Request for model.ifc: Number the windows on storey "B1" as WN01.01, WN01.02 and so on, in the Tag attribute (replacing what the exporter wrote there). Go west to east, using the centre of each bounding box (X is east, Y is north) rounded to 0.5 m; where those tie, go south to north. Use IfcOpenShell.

First a look at what the model holds.

```python
import ifcopenshell
import ifcopenshell.util.element
import ifcopenshell.util.placement

model = ifcopenshell.open("model.ifc")
print(model.schema)
storey = next(s for s in model.by_type("IfcBuildingStorey") if s.Name == "B1")
windows = [e for e in ifcopenshell.util.element.get_decomposition(storey) if e.is_a("IfcWindow")]
for e in sorted(windows, key=lambda e: e.id()):
    origin = ifcopenshell.util.placement.get_local_placement(e.ObjectPlacement)[:3, 3]
    print(e.id(), e.Tag, e.Name, origin.round(2) + 0.0, sep=" | ")
```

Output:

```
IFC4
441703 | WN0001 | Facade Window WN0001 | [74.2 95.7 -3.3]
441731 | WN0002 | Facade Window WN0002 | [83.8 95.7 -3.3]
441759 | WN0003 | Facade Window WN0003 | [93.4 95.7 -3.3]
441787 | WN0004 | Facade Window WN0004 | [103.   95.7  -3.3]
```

```python
import ifcopenshell
import ifcopenshell.geom
import ifcopenshell.util.element
import ifcopenshell.util.shape

model = ifcopenshell.open("model.ifc")
settings = ifcopenshell.geom.settings()
settings.set("use-world-coords", True)


def centre(element):
    shape = ifcopenshell.geom.create_shape(settings, element)
    return ifcopenshell.util.shape.get_bbox_centroid(shape.geometry)


storey = next(s for s in model.by_type("IfcBuildingStorey") if s.Name == "B1")
windows = [e for e in ifcopenshell.util.element.get_decomposition(storey) if e.is_a("IfcWindow")]

# Insertion points can sit at a corner or the storey origin, so sort by the geometry (in metres).
centres = {e: centre(e) for e in windows}
windows.sort(key=lambda e: (round(centres[e][0] / 0.5), centres[e][1]))

for i, e in enumerate(windows, start=1):
    number = f"WN01.{i:02d}"
    e.Tag = number
    print(e.id(), number)

model.write("model_edited.ifc")
```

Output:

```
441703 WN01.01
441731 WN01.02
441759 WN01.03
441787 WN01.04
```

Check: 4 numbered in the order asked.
